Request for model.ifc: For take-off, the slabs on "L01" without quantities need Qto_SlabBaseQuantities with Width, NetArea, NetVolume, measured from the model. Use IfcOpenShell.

First a look at what the model holds.

```python
import ifcopenshell
import ifcopenshell.util.element
import ifcopenshell.util.unit

model = ifcopenshell.open("model.ifc")
print(model.schema)
for unit_type in ("LENGTHUNIT", "AREAUNIT", "VOLUMEUNIT"):
    print(unit_type, ifcopenshell.util.unit.calculate_unit_scale(model, unit_type))
storey = next(s for s in model.by_type("IfcBuildingStorey") if s.Name == "L01")
slabs = [e for e in ifcopenshell.util.element.get_decomposition(storey) if e.is_a("IfcSlab")]
for e in sorted(slabs, key=lambda e: e.id()):
    print(e.id(), e.is_a(), e.Name, list(ifcopenshell.util.element.get_psets(e, qtos_only=True)), sep=" | ")
```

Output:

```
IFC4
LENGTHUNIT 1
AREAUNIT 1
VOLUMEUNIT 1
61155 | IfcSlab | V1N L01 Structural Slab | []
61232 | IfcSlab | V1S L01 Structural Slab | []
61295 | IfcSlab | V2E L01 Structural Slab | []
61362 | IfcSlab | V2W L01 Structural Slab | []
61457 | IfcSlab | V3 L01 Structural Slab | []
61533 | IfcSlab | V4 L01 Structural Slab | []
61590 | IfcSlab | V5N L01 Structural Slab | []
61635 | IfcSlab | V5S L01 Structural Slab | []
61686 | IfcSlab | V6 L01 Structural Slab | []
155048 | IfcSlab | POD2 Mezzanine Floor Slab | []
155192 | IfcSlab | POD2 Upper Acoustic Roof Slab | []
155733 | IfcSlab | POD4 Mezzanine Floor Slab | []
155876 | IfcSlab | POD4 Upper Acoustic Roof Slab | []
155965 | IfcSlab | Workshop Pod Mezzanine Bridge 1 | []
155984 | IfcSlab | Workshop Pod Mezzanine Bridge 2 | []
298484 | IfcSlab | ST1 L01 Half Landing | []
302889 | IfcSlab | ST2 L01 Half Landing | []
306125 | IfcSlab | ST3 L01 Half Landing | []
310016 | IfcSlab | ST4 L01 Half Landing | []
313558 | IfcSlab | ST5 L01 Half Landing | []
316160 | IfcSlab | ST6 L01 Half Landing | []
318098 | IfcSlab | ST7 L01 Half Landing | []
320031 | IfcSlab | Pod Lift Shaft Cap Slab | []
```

```python
import ifcopenshell
import ifcopenshell.api.pset
import ifcopenshell.geom
import ifcopenshell.util.element
import ifcopenshell.util.shape
import ifcopenshell.util.unit

model = ifcopenshell.open("model.ifc")
unit_scale = ifcopenshell.util.unit.calculate_unit_scale(model)
area_scale = ifcopenshell.util.unit.calculate_unit_scale(model, "AREAUNIT")
volume_scale = ifcopenshell.util.unit.calculate_unit_scale(model, "VOLUMEUNIT")
settings = ifcopenshell.geom.settings()

storey = next(s for s in model.by_type("IfcBuildingStorey") if s.Name == "L01")
slabs = [e for e in ifcopenshell.util.element.get_decomposition(storey) if e.is_a("IfcSlab")]

for e in sorted(slabs, key=lambda e: e.id()):
    if ifcopenshell.util.element.get_psets(e, qtos_only=True, should_inherit=False):
        continue
    # Geometry comes back in metres, in the element's own axes.
    shape = ifcopenshell.geom.create_shape(settings, e)
    values = {
        "Width": ifcopenshell.util.shape.get_z(shape.geometry) / unit_scale,
        "NetArea": ifcopenshell.util.shape.get_footprint_area(shape.geometry) / area_scale,
        "NetVolume": ifcopenshell.util.shape.get_volume(shape.geometry) / volume_scale,
    }
    qto = ifcopenshell.api.pset.add_qto(model, product=e, name="Qto_SlabBaseQuantities")
    ifcopenshell.api.pset.edit_qto(model, qto=qto, properties=values)
    print(e.id(), {k: round(v, 3) for k, v in values.items()})

model.write("model_rev.ifc")
```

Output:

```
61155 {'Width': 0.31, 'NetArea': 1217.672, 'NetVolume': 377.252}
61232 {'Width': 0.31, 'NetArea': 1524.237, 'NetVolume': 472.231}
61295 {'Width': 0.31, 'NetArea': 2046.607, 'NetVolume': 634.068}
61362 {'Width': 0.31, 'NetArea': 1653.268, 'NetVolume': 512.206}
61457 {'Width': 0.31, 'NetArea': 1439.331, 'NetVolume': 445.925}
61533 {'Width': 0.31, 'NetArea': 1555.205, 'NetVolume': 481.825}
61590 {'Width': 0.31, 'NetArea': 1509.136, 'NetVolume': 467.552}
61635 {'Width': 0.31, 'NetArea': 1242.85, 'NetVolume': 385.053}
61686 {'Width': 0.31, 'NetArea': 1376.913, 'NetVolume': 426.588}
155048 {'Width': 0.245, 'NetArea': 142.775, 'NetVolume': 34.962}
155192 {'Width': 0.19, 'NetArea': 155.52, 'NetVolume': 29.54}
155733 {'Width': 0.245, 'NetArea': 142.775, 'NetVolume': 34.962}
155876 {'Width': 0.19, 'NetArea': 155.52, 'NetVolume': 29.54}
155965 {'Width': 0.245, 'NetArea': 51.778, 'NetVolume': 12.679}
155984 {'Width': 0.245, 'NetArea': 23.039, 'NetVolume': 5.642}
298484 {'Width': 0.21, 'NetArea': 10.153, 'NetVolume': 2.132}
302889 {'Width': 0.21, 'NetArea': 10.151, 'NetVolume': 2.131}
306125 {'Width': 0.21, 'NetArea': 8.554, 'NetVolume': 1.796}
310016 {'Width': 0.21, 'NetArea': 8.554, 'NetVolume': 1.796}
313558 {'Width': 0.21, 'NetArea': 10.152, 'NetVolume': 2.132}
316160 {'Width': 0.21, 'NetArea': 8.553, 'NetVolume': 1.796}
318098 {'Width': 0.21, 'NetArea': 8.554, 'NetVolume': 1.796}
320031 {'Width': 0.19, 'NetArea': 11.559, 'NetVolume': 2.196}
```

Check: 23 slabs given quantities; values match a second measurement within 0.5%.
